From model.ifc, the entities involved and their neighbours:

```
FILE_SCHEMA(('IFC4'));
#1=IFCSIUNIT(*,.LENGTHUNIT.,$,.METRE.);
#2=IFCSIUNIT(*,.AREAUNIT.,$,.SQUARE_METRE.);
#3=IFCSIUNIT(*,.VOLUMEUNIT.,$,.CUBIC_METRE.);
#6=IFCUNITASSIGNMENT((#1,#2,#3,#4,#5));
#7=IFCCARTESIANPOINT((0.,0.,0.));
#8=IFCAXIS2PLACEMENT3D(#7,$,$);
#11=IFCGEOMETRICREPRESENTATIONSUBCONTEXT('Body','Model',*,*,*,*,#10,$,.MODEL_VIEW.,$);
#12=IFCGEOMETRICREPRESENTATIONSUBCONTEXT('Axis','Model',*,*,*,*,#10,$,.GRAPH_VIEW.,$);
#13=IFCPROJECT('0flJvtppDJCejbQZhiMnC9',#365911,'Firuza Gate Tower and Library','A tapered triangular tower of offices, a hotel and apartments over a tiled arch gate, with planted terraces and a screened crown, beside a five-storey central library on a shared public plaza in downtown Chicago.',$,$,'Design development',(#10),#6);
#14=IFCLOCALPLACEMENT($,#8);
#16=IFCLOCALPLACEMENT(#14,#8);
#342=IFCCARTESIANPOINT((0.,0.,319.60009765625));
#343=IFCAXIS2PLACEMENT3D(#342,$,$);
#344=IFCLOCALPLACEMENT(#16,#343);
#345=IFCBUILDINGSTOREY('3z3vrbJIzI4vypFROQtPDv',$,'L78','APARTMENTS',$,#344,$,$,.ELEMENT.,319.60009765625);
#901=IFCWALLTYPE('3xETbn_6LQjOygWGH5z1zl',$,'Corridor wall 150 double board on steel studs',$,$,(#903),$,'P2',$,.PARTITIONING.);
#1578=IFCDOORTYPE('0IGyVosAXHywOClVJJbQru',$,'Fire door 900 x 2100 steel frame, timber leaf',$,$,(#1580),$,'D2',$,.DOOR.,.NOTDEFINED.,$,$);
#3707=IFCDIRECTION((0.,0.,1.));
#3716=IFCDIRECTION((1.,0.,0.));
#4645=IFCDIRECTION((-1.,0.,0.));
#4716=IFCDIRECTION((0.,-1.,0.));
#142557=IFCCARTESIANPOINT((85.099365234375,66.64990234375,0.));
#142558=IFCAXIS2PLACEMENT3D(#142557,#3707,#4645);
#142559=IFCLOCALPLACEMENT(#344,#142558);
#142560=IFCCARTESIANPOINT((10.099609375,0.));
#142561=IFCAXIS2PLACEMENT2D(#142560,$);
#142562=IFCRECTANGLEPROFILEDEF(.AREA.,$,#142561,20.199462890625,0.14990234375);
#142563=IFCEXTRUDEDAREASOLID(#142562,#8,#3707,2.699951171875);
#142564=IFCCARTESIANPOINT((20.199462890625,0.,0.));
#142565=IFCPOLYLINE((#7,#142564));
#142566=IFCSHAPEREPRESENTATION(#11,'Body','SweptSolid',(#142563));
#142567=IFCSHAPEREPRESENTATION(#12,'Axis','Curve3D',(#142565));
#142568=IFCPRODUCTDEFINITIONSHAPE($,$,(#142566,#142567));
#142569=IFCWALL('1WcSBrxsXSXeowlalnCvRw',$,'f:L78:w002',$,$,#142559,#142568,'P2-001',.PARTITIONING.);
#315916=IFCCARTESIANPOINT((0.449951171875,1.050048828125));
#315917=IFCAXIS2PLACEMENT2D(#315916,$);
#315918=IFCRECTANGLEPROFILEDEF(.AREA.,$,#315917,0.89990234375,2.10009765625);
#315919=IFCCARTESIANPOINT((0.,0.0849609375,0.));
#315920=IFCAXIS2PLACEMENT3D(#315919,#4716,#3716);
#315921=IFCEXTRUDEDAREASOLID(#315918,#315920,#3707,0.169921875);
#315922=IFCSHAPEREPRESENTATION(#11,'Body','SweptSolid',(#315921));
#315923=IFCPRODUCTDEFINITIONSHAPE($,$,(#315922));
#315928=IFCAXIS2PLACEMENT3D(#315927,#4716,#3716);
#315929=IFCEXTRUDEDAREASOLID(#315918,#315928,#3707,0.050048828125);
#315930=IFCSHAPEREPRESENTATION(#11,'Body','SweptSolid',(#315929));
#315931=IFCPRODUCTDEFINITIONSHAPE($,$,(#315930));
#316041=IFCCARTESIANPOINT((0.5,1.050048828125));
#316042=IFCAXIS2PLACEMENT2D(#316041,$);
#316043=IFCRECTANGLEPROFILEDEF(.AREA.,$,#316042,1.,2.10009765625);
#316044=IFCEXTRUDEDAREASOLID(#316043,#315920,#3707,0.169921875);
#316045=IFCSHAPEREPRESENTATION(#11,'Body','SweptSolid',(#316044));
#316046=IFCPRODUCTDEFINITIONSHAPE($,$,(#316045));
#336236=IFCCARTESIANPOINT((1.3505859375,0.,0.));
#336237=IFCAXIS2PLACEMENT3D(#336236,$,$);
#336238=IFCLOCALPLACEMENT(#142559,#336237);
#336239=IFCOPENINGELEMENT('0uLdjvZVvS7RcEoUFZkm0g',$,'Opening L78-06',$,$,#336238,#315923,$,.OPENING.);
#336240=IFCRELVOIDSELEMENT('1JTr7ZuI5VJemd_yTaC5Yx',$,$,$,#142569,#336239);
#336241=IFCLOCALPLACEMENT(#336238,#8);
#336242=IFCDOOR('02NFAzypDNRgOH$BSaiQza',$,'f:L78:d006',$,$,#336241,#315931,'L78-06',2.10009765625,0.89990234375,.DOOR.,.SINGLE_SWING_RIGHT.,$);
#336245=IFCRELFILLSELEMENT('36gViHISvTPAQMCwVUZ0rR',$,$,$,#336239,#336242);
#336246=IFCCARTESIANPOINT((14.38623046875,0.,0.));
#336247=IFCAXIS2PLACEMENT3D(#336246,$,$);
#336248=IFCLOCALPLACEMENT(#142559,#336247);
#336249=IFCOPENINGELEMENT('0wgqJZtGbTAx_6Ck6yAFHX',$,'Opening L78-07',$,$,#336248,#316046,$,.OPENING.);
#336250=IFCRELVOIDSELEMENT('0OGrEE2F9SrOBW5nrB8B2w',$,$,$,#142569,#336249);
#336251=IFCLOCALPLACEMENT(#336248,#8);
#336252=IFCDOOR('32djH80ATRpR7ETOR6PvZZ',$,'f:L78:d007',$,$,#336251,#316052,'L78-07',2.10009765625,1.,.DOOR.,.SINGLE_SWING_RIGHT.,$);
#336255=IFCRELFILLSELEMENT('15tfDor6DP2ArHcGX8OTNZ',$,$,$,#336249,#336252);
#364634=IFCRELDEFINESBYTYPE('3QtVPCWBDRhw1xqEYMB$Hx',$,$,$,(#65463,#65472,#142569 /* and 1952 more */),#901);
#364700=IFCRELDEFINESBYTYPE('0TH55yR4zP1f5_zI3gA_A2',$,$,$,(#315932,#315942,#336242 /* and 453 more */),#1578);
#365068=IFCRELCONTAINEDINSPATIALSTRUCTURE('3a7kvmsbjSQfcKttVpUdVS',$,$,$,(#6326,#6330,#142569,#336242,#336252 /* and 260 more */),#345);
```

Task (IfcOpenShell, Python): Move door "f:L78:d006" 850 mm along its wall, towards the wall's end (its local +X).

```python
import ifcopenshell
import ifcopenshell.api.geometry
import ifcopenshell.util.placement

model = ifcopenshell.open("model.ifc")

door = model.by_id(336242)
opening = door.FillsVoids[0].RelatingOpeningElement
wall = opening.VoidsElements[0].RelatingBuildingElement

wall_matrix = ifcopenshell.util.placement.get_local_placement(wall.ObjectPlacement)
shift = wall_matrix[:3, 0] * 0.85
before = ifcopenshell.util.placement.get_local_placement(door.ObjectPlacement)[:3, 3].copy()

# The door is placed relative to its opening, so it follows when the opening moves.
matrix = ifcopenshell.util.placement.get_local_placement(opening.ObjectPlacement)
matrix[:3, 3] += shift
ifcopenshell.api.geometry.edit_object_placement(
    model, product=opening, matrix=matrix, is_si=False, should_transform_children=True
)

after = ifcopenshell.util.placement.get_local_placement(door.ObjectPlacement)[:3, 3]
print("door moved by", (after - before).round(3) + 0.0)

model.write("model_edited.ifc")
```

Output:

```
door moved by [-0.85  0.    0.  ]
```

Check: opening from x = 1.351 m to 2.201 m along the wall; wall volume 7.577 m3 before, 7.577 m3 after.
